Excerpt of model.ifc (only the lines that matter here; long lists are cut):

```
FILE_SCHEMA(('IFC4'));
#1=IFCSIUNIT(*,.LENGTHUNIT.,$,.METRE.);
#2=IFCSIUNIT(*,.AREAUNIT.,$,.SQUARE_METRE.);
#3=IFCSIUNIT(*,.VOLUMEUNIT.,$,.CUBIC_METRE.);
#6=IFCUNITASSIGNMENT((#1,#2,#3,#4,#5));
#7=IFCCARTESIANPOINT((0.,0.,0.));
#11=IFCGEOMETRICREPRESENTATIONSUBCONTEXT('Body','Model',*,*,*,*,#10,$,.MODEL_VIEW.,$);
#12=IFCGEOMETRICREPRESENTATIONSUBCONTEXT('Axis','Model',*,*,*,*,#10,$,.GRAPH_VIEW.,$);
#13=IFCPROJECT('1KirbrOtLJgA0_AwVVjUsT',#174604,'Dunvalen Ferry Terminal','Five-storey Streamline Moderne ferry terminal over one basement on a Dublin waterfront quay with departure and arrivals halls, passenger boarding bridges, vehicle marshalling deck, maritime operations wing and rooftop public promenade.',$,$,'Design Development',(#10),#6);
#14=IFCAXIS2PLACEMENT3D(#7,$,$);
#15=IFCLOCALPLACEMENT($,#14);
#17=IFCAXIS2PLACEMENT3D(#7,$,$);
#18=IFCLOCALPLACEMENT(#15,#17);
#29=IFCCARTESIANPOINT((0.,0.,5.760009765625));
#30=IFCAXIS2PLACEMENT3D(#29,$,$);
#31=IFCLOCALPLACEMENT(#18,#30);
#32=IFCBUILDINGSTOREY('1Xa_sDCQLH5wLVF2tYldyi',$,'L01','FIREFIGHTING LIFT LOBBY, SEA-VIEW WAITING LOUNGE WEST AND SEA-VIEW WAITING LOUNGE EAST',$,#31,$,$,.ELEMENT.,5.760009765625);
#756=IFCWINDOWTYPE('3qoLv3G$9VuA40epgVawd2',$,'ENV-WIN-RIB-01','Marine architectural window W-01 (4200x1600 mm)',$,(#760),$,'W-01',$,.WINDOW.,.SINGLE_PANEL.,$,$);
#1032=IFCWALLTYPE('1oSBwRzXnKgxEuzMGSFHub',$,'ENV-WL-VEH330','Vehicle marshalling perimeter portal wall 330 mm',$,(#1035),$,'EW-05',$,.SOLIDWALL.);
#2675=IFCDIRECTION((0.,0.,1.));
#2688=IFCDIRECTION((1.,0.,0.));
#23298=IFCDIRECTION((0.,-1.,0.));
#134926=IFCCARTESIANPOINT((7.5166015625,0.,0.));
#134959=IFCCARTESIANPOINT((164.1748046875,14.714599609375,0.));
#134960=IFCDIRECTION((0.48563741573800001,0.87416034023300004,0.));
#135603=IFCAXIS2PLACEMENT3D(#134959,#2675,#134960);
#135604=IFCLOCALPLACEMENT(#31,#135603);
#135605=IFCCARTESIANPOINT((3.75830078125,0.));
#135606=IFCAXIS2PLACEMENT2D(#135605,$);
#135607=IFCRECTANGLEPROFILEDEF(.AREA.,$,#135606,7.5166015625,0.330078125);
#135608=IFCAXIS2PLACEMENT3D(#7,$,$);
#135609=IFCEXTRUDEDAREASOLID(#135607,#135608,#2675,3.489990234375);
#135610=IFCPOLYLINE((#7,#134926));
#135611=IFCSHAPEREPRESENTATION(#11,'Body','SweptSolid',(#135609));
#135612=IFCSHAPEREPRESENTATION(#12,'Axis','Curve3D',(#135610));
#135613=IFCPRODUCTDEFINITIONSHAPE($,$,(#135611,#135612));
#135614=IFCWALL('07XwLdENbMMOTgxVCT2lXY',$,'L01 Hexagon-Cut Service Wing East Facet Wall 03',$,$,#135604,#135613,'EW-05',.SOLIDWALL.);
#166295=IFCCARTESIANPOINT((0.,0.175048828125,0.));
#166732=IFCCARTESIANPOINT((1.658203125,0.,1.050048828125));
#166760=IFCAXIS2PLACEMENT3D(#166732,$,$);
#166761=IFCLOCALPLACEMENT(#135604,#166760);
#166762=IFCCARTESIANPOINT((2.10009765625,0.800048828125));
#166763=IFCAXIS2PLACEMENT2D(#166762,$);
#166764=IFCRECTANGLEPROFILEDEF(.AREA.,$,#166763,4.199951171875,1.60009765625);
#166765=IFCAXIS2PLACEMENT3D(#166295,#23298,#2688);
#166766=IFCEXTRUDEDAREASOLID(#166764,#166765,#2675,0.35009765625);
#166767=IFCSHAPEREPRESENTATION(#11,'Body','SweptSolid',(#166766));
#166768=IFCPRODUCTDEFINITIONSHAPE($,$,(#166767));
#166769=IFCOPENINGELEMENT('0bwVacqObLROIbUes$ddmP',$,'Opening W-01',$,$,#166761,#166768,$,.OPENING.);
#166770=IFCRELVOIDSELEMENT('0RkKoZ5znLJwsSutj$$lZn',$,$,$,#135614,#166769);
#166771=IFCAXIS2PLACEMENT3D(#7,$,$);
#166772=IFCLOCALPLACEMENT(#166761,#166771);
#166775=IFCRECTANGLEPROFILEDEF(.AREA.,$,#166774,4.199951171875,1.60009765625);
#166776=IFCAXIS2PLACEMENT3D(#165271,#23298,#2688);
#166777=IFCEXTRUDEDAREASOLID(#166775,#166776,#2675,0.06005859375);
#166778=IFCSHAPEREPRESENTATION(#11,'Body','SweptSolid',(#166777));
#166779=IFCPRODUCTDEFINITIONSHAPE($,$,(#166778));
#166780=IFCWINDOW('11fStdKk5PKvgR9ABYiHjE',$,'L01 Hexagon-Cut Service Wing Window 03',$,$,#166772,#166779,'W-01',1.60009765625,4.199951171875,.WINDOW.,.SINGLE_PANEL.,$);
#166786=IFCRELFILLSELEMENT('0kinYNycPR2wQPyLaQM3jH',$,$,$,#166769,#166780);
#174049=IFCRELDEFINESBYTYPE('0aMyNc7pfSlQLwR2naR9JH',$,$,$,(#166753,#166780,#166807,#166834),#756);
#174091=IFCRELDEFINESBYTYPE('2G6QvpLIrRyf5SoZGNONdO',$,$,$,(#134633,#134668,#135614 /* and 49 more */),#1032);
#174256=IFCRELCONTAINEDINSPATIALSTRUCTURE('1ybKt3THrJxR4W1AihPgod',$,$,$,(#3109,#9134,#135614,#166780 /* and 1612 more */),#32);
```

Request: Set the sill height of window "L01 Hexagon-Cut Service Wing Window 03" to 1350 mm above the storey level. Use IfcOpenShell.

```python
import numpy as np
import ifcopenshell
import ifcopenshell.api.geometry
import ifcopenshell.geom
import ifcopenshell.util.element
import ifcopenshell.util.placement
import ifcopenshell.util.shape
import ifcopenshell.util.unit

model = ifcopenshell.open("model.ifc")
unit_scale = ifcopenshell.util.unit.calculate_unit_scale(model)

window = model.by_guid("11fStdKk5PKvgR9ABYiHjE")
opening = window.FillsVoids[0].RelatingOpeningElement
storey = ifcopenshell.util.element.get_container(window, ifc_class="IfcBuildingStorey")
level = ifcopenshell.util.placement.get_local_placement(storey.ObjectPlacement)[2, 3]

# The opening's origin need not be at the sill, so measure its lowest point.
shape = ifcopenshell.geom.create_shape(ifcopenshell.geom.settings(), opening)
bottom = ifcopenshell.util.shape.get_shape_bottom_elevation(shape, shape.geometry) / unit_scale
dz = level + 1.35 / unit_scale - bottom

shift = np.array([0.0, 0.0, dz])
# The window is placed relative to its opening, so it follows when the opening moves.
matrix = ifcopenshell.util.placement.get_local_placement(opening.ObjectPlacement)
matrix[:3, 3] += shift
ifcopenshell.api.geometry.edit_object_placement(
    model, product=opening, matrix=matrix, is_si=False, should_transform_children=True
)

print(f"moved by {dz * unit_scale:+.3f} m")

model.write("model_updated.ifc")
```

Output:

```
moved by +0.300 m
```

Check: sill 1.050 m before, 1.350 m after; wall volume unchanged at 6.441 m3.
